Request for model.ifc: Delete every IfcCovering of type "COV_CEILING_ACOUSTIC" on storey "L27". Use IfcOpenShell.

First a look at what the model holds.

```python
import ifcopenshell
import ifcopenshell.util.element

model = ifcopenshell.open("model.ifc")
print(model.schema)
storey = next(s for s in model.by_type("IfcBuildingStorey") if s.Name == "L27")
coverings = [e for e in ifcopenshell.util.element.get_decomposition(storey) if e.is_a("IfcCovering")]
seen = {}
for e in coverings:
    element_type = ifcopenshell.util.element.get_type(e)
    name = element_type.Name if element_type not in (None, e) else None
    seen[name] = seen.get(name, 0) + 1
for name, count in sorted(seen.items(), key=str):
    print(count, "x", name)
```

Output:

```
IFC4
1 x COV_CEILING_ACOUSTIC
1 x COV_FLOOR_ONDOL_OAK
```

```python
import ifcopenshell
import ifcopenshell.api.root
import ifcopenshell.util.element

model = ifcopenshell.open("model.ifc")

storey = next(s for s in model.by_type("IfcBuildingStorey") if s.Name == "L27")
coverings = [e for e in ifcopenshell.util.element.get_decomposition(storey) if e.is_a("IfcCovering")]
targets = [e for e in coverings if (t := ifcopenshell.util.element.get_type(e)) not in (None, e) and t.Name == "COV_CEILING_ACOUSTIC"]

for e in targets:
    ifcopenshell.api.root.remove_product(model, product=e)
print(len(targets), "removed")

model.write("model_v2.ifc")
```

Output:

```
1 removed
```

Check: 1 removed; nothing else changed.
